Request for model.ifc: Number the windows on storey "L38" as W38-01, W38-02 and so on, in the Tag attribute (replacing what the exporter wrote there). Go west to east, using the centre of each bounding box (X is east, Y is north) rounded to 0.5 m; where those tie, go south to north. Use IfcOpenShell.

First a look at what the model holds.

```python
import ifcopenshell
import ifcopenshell.util.element
import ifcopenshell.util.placement

model = ifcopenshell.open("model.ifc")
print(model.schema)
storey = next(s for s in model.by_type("IfcBuildingStorey") if s.Name == "L38")
windows = [e for e in ifcopenshell.util.element.get_decomposition(storey) if e.is_a("IfcWindow")]
for e in sorted(windows, key=lambda e: e.id()):
    origin = ifcopenshell.util.placement.get_local_placement(e.ObjectPlacement)[:3, 3]
    print(e.id(), e.Tag, e.Name, origin.round(2) + 0.0, sep=" | ")
```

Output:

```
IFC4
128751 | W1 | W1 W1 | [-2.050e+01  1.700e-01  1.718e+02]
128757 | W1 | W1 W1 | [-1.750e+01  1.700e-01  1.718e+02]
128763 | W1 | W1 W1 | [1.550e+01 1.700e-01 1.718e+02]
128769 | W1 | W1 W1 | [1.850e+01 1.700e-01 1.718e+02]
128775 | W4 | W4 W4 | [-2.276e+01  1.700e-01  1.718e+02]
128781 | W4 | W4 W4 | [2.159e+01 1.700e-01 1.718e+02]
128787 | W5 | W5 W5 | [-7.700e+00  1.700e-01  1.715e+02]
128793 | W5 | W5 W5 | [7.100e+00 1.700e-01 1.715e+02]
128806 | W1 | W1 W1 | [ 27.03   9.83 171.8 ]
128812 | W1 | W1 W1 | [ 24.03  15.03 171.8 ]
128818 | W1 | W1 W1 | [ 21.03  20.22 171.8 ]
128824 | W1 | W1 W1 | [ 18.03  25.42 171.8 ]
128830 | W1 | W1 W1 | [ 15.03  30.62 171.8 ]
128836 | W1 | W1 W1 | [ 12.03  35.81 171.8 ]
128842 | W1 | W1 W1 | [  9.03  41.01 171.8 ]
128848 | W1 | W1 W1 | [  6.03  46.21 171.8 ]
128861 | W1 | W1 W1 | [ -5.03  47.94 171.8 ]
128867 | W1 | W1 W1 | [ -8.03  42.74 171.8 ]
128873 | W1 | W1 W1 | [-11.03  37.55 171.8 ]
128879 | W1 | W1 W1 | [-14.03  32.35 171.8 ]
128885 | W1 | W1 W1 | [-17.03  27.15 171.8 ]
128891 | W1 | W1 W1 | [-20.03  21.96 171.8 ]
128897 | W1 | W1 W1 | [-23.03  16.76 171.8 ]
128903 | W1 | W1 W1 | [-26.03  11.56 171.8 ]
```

```python
import ifcopenshell
import ifcopenshell.geom
import ifcopenshell.util.element
import ifcopenshell.util.shape

model = ifcopenshell.open("model.ifc")
settings = ifcopenshell.geom.settings()
settings.set("use-world-coords", True)


def centre(element):
    shape = ifcopenshell.geom.create_shape(settings, element)
    return ifcopenshell.util.shape.get_bbox_centroid(shape.geometry)


storey = next(s for s in model.by_type("IfcBuildingStorey") if s.Name == "L38")
windows = [e for e in ifcopenshell.util.element.get_decomposition(storey) if e.is_a("IfcWindow")]

# Insertion points can sit at a corner or the storey origin, so sort by the geometry (in metres).
centres = {e: centre(e) for e in windows}
windows.sort(key=lambda e: (round(centres[e][0] / 0.5), centres[e][1]))

for i, e in enumerate(windows, start=1):
    number = f"W38-{i:02d}"
    e.Tag = number
    print(e.id(), number)

model.write("model-out.ifc")
```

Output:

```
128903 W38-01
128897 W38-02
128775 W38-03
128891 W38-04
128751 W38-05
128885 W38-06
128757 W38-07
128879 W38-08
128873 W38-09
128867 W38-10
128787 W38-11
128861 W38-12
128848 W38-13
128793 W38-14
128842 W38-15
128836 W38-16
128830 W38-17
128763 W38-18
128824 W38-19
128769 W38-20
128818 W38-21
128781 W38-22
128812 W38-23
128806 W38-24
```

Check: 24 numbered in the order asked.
